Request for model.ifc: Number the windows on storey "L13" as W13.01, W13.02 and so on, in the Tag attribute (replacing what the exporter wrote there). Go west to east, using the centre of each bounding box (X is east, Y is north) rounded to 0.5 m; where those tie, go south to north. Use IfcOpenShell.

First a look at what the model holds.

```python
import ifcopenshell
import ifcopenshell.util.element
import ifcopenshell.util.placement

model = ifcopenshell.open("model.ifc")
print(model.schema)
storey = next(s for s in model.by_type("IfcBuildingStorey") if s.Name == "L13")
windows = [e for e in ifcopenshell.util.element.get_decomposition(storey) if e.is_a("IfcWindow")]
for e in sorted(windows, key=lambda e: e.id()):
    origin = ifcopenshell.util.placement.get_local_placement(e.ObjectPlacement)[:3, 3]
    print(e.id(), e.Tag, e.Name, origin.round(2) + 0.0, sep=" | ")
```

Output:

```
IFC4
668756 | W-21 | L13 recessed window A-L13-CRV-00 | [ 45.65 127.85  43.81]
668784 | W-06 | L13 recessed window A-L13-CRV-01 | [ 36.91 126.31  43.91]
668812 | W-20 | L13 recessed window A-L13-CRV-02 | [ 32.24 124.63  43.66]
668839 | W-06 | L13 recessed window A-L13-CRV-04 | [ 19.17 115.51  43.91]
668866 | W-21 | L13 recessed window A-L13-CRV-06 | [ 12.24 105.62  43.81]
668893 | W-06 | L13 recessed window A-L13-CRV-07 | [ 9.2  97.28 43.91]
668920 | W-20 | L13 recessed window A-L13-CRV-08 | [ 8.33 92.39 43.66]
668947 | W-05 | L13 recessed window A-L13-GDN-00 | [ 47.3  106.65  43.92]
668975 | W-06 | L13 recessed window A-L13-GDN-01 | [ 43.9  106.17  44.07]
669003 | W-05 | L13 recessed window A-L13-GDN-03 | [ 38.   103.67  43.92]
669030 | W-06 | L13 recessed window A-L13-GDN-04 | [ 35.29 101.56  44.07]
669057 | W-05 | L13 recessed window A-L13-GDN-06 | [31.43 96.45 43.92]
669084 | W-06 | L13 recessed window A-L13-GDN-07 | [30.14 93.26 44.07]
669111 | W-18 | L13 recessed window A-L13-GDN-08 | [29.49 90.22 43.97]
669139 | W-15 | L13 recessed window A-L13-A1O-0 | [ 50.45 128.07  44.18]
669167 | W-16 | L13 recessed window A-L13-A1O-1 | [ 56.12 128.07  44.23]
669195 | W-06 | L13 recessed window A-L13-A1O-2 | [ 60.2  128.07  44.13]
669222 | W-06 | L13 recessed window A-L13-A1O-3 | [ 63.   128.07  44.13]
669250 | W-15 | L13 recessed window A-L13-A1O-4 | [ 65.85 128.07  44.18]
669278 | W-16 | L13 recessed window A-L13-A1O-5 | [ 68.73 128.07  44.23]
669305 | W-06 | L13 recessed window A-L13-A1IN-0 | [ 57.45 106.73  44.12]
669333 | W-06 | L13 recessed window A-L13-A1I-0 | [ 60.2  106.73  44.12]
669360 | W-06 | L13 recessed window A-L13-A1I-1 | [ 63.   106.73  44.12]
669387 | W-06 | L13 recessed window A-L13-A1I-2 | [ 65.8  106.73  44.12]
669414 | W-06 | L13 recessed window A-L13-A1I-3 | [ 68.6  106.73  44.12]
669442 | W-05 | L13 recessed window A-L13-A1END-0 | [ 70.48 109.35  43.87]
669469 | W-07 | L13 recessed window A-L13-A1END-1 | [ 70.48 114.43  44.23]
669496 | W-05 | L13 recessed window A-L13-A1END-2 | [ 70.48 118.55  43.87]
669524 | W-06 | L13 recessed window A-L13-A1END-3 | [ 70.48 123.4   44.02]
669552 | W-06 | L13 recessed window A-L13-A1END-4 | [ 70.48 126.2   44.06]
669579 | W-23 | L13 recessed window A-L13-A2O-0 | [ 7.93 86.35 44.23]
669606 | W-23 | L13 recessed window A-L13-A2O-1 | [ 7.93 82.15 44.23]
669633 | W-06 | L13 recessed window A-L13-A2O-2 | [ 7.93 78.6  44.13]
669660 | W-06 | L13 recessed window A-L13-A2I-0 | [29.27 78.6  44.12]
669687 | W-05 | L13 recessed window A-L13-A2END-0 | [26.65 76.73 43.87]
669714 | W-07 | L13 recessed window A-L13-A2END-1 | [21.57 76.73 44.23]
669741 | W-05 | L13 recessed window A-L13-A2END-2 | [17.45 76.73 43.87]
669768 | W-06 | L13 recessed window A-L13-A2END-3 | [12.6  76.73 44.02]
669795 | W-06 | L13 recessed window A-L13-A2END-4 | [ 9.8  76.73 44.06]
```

```python
import ifcopenshell
import ifcopenshell.geom
import ifcopenshell.util.element
import ifcopenshell.util.shape

model = ifcopenshell.open("model.ifc")
settings = ifcopenshell.geom.settings()
settings.set("use-world-coords", True)


def centre(element):
    shape = ifcopenshell.geom.create_shape(settings, element)
    return ifcopenshell.util.shape.get_bbox_centroid(shape.geometry)


storey = next(s for s in model.by_type("IfcBuildingStorey") if s.Name == "L13")
windows = [e for e in ifcopenshell.util.element.get_decomposition(storey) if e.is_a("IfcWindow")]

# Insertion points can sit at a corner or the storey origin, so sort by the geometry (in metres).
centres = {e: centre(e) for e in windows}
windows.sort(key=lambda e: (round(centres[e][0] / 0.5), centres[e][1]))

for i, e in enumerate(windows, start=1):
    number = f"W13.{i:02d}"
    e.Tag = number
    print(e.id(), number)

model.write("model_updated.ifc")
```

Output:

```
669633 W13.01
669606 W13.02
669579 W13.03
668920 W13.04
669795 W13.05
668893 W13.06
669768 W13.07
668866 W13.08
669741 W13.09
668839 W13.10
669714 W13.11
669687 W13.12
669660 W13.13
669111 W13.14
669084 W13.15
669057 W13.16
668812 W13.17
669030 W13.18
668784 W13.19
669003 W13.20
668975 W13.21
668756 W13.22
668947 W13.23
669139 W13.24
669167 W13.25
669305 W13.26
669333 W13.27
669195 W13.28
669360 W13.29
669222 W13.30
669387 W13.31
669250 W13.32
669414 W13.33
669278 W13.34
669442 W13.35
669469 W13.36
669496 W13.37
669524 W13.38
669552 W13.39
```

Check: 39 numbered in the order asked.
